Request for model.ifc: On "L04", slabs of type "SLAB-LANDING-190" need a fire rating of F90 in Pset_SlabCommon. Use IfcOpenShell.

First a look at what the model holds.

```python
import ifcopenshell
import ifcopenshell.util.element

model = ifcopenshell.open("model.ifc")
print(model.schema)
storey = next(s for s in model.by_type("IfcBuildingStorey") if s.Name == "L04")
slabs = [e for e in ifcopenshell.util.element.get_decomposition(storey) if e.is_a("IfcSlab")]
seen = {}
for e in slabs:
    element_type = ifcopenshell.util.element.get_type(e)
    key = (element_type.Name if element_type != e and element_type else None, ifcopenshell.util.element.get_pset(e, "Pset_SlabCommon", "FireRating"))
    seen[key] = seen.get(key, 0) + 1
for (name, value), count in sorted(seen.items(), key=str):
    print(count, "x", name, "|", value)
```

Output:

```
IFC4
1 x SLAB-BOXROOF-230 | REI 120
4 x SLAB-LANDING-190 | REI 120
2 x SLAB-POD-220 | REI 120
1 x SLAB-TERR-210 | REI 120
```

```python
import ifcopenshell
import ifcopenshell.api.pset
import ifcopenshell.util.element

model = ifcopenshell.open("model.ifc")

storey = next(s for s in model.by_type("IfcBuildingStorey") if s.Name == "L04")
slabs = [e for e in ifcopenshell.util.element.get_decomposition(storey) if e.is_a("IfcSlab")]

count = 0
for e in slabs:
    element_type = ifcopenshell.util.element.get_type(e)
    if element_type in (None, e) or element_type.Name != "SLAB-LANDING-190":
        continue
    # add_pset returns the element's existing set when there is one.
    pset = ifcopenshell.api.pset.add_pset(model, product=e, name="Pset_SlabCommon")
    ifcopenshell.api.pset.edit_pset(model, pset=pset, properties={"FireRating": "F90"})
    count += 1

print(count, "slabs updated")

model.write("model-out.ifc")
```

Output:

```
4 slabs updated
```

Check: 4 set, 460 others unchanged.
